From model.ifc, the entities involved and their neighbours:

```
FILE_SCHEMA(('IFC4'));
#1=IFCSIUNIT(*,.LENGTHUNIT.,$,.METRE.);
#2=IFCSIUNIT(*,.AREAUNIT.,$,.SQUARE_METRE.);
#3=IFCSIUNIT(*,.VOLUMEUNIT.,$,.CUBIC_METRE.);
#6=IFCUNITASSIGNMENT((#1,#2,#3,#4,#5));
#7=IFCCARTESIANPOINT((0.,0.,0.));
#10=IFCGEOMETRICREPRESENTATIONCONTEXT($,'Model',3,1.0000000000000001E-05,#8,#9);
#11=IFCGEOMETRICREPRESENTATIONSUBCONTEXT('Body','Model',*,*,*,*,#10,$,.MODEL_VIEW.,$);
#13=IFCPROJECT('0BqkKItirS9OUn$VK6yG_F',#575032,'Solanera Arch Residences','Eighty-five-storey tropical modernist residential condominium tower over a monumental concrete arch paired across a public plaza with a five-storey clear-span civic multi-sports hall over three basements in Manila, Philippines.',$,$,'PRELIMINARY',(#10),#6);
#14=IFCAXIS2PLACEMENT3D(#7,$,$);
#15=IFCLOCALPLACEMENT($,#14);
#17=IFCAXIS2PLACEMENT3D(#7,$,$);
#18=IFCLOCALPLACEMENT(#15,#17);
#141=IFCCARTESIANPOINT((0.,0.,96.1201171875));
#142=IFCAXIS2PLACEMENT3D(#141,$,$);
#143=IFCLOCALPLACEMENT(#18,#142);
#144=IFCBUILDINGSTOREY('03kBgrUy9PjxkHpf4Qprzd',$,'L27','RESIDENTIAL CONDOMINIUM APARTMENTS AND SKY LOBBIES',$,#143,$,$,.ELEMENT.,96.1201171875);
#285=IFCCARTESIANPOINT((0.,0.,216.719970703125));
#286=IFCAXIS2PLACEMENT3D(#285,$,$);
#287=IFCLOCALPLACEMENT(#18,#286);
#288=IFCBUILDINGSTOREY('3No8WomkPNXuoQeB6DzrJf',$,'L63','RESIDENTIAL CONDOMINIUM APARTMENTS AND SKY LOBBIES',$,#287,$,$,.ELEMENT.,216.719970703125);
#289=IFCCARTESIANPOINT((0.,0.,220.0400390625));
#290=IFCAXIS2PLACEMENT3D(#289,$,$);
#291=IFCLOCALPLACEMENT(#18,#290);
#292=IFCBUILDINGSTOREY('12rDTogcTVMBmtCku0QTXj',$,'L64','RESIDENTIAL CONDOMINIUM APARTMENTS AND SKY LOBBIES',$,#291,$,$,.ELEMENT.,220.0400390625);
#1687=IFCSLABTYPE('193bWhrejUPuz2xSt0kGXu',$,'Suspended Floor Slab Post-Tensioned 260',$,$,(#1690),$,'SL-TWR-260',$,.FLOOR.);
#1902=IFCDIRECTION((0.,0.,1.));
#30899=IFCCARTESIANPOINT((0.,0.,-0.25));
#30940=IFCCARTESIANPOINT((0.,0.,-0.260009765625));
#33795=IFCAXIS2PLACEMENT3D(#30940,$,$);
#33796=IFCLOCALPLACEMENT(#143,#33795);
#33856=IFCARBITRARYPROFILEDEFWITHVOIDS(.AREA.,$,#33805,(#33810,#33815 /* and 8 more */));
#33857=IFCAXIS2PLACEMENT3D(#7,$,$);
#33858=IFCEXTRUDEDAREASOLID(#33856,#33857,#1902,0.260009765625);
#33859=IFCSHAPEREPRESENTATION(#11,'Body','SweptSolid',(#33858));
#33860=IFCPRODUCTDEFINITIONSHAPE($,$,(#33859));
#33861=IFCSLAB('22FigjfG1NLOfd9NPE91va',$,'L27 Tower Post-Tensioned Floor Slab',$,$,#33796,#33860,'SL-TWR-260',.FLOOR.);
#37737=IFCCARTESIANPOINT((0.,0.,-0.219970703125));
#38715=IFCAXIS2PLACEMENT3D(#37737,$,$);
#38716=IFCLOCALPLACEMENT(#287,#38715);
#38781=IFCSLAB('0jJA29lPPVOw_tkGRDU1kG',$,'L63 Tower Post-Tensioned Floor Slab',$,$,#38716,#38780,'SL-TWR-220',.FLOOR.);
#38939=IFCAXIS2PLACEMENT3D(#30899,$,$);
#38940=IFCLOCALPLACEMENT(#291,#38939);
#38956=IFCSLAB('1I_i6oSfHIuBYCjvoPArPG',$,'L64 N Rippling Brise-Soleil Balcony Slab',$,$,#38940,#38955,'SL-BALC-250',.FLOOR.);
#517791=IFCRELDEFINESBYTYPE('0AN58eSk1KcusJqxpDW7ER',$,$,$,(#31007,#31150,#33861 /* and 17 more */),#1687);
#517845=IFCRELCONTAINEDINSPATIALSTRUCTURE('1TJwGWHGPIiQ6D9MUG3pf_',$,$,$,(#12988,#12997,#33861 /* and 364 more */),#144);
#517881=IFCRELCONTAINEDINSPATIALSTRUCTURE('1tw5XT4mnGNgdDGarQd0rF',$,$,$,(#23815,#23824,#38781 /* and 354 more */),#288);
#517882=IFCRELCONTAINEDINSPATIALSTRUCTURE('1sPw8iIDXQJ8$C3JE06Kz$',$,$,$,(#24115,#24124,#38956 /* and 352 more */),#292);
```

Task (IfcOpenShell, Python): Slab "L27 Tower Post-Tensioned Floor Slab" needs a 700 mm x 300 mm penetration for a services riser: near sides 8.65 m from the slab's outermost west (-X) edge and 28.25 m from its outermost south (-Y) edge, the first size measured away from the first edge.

```python
import numpy as np
import ifcopenshell
import ifcopenshell.api.feature
import ifcopenshell.api.geometry
import ifcopenshell.api.root
import ifcopenshell.geom
import ifcopenshell.util.placement
import ifcopenshell.util.representation
import ifcopenshell.util.shape
import ifcopenshell.util.unit

model = ifcopenshell.open("model.ifc")
unit_scale = ifcopenshell.util.unit.calculate_unit_scale(model)
settings = ifcopenshell.geom.settings()


def volume(element):
    """Net volume in cubic metres, openings subtracted."""
    shape = ifcopenshell.geom.create_shape(settings, element)
    return ifcopenshell.util.shape.get_volume(shape.geometry)


slab = model.by_guid("22FigjfG1NLOfd9NPE91va")
before = volume(slab)

# Extent in the slab's own axes, in metres. The edges named are its -X and -Y sides.
slab_shape = ifcopenshell.geom.create_shape(settings, slab)
vertices = ifcopenshell.util.shape.get_vertices(slab_shape.geometry)
x_min, y_min, bottom = vertices.min(axis=0)
top = vertices[:, 2].max()

opening = ifcopenshell.api.root.create_entity(model, ifc_class="IfcOpeningElement", name="Services riser opening", predefined_type="OPENING")
context = ifcopenshell.util.representation.get_context(model, "Model", "Body", "MODEL_VIEW")
width, depth = 0.7, 0.3
outline = [(0.0, 0.0), (width, 0.0), (width, depth), (0.0, depth), (0.0, 0.0)]
# Overshoot both faces by 50 mm so the cut is clean.
shape = ifcopenshell.api.geometry.add_slab_representation(
    model, context=context, depth=top - bottom + 0.1, polyline=outline
)
ifcopenshell.api.geometry.assign_representation(model, product=opening, representation=shape)

matrix = ifcopenshell.util.placement.get_local_placement(slab.ObjectPlacement)
matrix[:, 3] = matrix @ np.append(np.array([x_min + 8.65, y_min + 28.25, bottom - 0.05]) / unit_scale, 1.0)
ifcopenshell.api.geometry.edit_object_placement(model, product=opening, matrix=matrix, is_si=False)
ifcopenshell.api.feature.add_feature(model, feature=opening, element=slab)

after = volume(slab)

print(f"slab volume {before:.3f} -> {after:.3f} m3")

model.write("model_edited.ifc")
```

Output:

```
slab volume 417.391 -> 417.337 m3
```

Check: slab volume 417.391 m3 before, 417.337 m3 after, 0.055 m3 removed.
